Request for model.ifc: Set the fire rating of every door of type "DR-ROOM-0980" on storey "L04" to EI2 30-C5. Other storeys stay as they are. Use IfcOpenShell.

First a look at what the model holds.

```python
import ifcopenshell
import ifcopenshell.util.element

model = ifcopenshell.open("model.ifc")
print(model.schema)
storey = next(s for s in model.by_type("IfcBuildingStorey") if s.Name == "L04")
doors = [e for e in ifcopenshell.util.element.get_decomposition(storey) if e.is_a("IfcDoor")]
seen = {}
for e in doors:
    element_type = ifcopenshell.util.element.get_type(e)
    key = (element_type.Name if element_type != e and element_type else None, ifcopenshell.util.element.get_pset(e, "Pset_DoorCommon", "FireRating"))
    seen[key] = seen.get(key, 0) + 1
for (name, value), count in sorted(seen.items(), key=str):
    print(count, "x", name, "|", value)
```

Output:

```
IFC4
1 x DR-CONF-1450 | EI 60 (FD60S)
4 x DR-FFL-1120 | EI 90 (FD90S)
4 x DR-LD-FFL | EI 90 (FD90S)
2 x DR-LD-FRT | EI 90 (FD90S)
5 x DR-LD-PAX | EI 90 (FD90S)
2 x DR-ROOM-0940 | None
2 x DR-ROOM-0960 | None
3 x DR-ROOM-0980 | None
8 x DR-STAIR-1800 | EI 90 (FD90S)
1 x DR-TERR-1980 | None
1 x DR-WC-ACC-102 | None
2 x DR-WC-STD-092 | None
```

```python
import ifcopenshell
import ifcopenshell.api.pset
import ifcopenshell.util.element

model = ifcopenshell.open("model.ifc")

storey = next(s for s in model.by_type("IfcBuildingStorey") if s.Name == "L04")
doors = [e for e in ifcopenshell.util.element.get_decomposition(storey) if e.is_a("IfcDoor")]

count = 0
for e in doors:
    element_type = ifcopenshell.util.element.get_type(e)
    if element_type in (None, e) or element_type.Name != "DR-ROOM-0980":
        continue
    # add_pset returns the element's existing set when there is one.
    pset = ifcopenshell.api.pset.add_pset(model, product=e, name="Pset_DoorCommon")
    ifcopenshell.api.pset.edit_pset(model, pset=pset, properties={"FireRating": "EI2 30-C5"})
    count += 1

print(count, "doors updated")

model.write("model_updated.ifc")
```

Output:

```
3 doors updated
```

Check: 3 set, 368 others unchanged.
